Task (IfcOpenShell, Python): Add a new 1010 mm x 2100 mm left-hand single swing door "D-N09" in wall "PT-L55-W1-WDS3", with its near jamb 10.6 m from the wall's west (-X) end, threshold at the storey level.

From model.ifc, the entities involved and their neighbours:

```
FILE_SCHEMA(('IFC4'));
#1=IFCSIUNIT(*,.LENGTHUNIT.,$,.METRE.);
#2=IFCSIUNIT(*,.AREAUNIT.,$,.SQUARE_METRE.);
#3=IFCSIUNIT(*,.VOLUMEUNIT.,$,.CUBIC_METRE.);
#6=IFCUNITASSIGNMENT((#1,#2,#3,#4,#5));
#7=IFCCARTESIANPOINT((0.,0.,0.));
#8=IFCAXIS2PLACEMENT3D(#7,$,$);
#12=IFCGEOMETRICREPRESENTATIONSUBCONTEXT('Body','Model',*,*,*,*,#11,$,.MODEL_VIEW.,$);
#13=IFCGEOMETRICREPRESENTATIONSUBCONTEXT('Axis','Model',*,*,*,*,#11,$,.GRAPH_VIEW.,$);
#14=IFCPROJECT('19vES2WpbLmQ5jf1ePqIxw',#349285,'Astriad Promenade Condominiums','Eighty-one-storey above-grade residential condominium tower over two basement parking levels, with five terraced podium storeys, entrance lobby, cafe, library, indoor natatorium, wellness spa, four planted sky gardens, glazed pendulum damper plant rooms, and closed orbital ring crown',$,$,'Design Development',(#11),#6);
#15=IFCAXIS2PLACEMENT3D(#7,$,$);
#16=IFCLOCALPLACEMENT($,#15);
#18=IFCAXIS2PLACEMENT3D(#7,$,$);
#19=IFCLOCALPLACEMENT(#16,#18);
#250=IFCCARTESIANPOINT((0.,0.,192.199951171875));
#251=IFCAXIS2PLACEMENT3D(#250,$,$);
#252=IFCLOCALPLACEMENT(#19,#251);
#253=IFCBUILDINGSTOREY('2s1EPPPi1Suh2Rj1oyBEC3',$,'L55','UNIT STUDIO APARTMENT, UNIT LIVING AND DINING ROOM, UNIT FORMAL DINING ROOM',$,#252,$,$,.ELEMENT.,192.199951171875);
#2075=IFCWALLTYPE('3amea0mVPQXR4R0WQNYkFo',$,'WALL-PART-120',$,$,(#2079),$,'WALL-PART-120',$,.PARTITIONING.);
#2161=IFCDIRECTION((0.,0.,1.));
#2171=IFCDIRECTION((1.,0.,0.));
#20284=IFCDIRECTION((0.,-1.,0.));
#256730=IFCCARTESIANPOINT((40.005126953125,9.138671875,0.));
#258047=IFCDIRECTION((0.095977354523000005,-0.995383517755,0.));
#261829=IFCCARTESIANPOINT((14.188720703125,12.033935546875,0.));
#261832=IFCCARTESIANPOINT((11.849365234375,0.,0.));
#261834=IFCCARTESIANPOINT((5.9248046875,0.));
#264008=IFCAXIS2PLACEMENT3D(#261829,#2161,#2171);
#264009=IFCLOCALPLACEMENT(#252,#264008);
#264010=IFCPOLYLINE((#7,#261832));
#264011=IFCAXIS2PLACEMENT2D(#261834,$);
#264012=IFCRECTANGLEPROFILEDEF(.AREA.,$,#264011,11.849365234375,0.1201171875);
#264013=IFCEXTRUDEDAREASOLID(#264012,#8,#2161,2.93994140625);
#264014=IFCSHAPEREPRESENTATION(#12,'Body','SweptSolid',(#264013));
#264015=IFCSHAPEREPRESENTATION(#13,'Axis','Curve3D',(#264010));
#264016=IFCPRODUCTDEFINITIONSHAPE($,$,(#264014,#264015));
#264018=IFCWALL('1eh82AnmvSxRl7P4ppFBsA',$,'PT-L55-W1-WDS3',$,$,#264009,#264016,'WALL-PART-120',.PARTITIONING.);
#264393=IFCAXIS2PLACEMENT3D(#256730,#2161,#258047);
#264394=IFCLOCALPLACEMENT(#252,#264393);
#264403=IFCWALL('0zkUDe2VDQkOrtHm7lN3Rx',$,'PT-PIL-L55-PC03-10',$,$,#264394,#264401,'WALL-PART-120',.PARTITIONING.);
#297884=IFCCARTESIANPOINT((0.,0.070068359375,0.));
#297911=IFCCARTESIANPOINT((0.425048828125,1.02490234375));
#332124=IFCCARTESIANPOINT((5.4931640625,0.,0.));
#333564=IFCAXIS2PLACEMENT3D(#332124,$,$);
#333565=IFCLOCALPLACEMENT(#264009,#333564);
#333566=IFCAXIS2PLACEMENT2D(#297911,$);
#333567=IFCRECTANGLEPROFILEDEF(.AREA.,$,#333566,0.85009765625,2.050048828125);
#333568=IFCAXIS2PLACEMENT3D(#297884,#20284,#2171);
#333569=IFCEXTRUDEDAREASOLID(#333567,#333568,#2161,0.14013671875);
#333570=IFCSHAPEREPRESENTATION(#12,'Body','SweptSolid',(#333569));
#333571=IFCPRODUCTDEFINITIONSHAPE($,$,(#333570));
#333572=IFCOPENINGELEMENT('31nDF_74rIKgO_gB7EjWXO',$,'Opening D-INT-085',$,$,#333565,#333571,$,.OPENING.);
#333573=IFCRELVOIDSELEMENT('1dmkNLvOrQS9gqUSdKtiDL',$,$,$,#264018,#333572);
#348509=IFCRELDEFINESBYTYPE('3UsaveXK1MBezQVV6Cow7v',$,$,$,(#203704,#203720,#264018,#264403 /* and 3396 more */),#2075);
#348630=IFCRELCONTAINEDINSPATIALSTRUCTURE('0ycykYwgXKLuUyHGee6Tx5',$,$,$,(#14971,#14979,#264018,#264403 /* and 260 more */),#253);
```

```python
import numpy as np
import ifcopenshell
import ifcopenshell.api.feature
import ifcopenshell.api.geometry
import ifcopenshell.api.root
import ifcopenshell.api.spatial
import ifcopenshell.geom
import ifcopenshell.util.element
import ifcopenshell.util.placement
import ifcopenshell.util.representation
import ifcopenshell.util.shape
import ifcopenshell.util.unit

model = ifcopenshell.open("model.ifc")
unit_scale = ifcopenshell.util.unit.calculate_unit_scale(model)
settings = ifcopenshell.geom.settings()


def volume(element):
    """Net volume in cubic metres, openings subtracted."""
    shape = ifcopenshell.geom.create_shape(settings, element)
    return ifcopenshell.util.shape.get_volume(shape.geometry)


wall = model.by_guid("1eh82AnmvSxRl7P4ppFBsA")
storey = ifcopenshell.util.element.get_container(wall, ifc_class="IfcBuildingStorey")
context = ifcopenshell.util.representation.get_context(model, "Model", "Body", "MODEL_VIEW")
before = volume(wall)

width, height, from_end, sill = 1.01, 2.1, 10.6, 0.0  # metres

# The wall runs along its own X axis, and the end named is its -X end.
wall_shape = ifcopenshell.geom.create_shape(settings, wall)
x, y, z = ifcopenshell.util.shape.get_vertices(wall_shape.geometry).T
start = x.min() + from_end
face, thickness = float(y.min()), float(y.max() - y.min())
wall_matrix = ifcopenshell.util.placement.get_local_placement(wall.ObjectPlacement)
level = ifcopenshell.util.placement.get_local_placement(storey.ObjectPlacement)[2, 3]


def in_wall(x, y):
    """Placement at x, y metres in the wall's axes, at sill height."""
    matrix = wall_matrix.copy()
    matrix[:, 3] = wall_matrix @ np.array([x / unit_scale, y / unit_scale, 0.0, 1.0])
    matrix[2, 3] = level + sill / unit_scale
    return matrix


# Opening: a box that overshoots both wall faces by 50 mm.
opening = ifcopenshell.api.root.create_entity(model, ifc_class="IfcOpeningElement", predefined_type="OPENING")
box = ifcopenshell.api.geometry.add_wall_representation(
    model, context=context, length=width, height=height, thickness=thickness + 0.1
)
ifcopenshell.api.geometry.assign_representation(model, product=opening, representation=box)
ifcopenshell.api.geometry.edit_object_placement(model, product=opening, matrix=in_wall(start, face - 0.05), is_si=False)
ifcopenshell.api.feature.add_feature(model, feature=opening, element=wall)

door = ifcopenshell.api.root.create_entity(model, ifc_class="IfcDoor", name="D-N09", predefined_type="DOOR")
door.OverallWidth, door.OverallHeight = width / unit_scale, height / unit_scale
door.OperationType = "SINGLE_SWING_LEFT"
body = ifcopenshell.api.geometry.add_door_representation(
    model,
    context=context,
    overall_width=door.OverallWidth,
    overall_height=door.OverallHeight,
    operation_type="SINGLE_SWING_LEFT",
    lining_properties={"LiningDepth": thickness / unit_scale, "ThresholdDepth": thickness / unit_scale},
)
ifcopenshell.api.geometry.assign_representation(model, product=door, representation=body)
ifcopenshell.api.spatial.assign_container(model, products=[door], relating_structure=storey)
ifcopenshell.api.feature.add_filling(model, opening=opening, element=door)

# The lining spans the wall, so the door starts at the wall face.
ifcopenshell.api.geometry.edit_object_placement(model, product=door, matrix=in_wall(start, face), is_si=False)

after = volume(wall)

print(f"wall volume {before:.3f} -> {after:.3f} m3")

model.write("model_rev.ifc")
```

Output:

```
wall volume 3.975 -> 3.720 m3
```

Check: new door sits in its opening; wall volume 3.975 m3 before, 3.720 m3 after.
